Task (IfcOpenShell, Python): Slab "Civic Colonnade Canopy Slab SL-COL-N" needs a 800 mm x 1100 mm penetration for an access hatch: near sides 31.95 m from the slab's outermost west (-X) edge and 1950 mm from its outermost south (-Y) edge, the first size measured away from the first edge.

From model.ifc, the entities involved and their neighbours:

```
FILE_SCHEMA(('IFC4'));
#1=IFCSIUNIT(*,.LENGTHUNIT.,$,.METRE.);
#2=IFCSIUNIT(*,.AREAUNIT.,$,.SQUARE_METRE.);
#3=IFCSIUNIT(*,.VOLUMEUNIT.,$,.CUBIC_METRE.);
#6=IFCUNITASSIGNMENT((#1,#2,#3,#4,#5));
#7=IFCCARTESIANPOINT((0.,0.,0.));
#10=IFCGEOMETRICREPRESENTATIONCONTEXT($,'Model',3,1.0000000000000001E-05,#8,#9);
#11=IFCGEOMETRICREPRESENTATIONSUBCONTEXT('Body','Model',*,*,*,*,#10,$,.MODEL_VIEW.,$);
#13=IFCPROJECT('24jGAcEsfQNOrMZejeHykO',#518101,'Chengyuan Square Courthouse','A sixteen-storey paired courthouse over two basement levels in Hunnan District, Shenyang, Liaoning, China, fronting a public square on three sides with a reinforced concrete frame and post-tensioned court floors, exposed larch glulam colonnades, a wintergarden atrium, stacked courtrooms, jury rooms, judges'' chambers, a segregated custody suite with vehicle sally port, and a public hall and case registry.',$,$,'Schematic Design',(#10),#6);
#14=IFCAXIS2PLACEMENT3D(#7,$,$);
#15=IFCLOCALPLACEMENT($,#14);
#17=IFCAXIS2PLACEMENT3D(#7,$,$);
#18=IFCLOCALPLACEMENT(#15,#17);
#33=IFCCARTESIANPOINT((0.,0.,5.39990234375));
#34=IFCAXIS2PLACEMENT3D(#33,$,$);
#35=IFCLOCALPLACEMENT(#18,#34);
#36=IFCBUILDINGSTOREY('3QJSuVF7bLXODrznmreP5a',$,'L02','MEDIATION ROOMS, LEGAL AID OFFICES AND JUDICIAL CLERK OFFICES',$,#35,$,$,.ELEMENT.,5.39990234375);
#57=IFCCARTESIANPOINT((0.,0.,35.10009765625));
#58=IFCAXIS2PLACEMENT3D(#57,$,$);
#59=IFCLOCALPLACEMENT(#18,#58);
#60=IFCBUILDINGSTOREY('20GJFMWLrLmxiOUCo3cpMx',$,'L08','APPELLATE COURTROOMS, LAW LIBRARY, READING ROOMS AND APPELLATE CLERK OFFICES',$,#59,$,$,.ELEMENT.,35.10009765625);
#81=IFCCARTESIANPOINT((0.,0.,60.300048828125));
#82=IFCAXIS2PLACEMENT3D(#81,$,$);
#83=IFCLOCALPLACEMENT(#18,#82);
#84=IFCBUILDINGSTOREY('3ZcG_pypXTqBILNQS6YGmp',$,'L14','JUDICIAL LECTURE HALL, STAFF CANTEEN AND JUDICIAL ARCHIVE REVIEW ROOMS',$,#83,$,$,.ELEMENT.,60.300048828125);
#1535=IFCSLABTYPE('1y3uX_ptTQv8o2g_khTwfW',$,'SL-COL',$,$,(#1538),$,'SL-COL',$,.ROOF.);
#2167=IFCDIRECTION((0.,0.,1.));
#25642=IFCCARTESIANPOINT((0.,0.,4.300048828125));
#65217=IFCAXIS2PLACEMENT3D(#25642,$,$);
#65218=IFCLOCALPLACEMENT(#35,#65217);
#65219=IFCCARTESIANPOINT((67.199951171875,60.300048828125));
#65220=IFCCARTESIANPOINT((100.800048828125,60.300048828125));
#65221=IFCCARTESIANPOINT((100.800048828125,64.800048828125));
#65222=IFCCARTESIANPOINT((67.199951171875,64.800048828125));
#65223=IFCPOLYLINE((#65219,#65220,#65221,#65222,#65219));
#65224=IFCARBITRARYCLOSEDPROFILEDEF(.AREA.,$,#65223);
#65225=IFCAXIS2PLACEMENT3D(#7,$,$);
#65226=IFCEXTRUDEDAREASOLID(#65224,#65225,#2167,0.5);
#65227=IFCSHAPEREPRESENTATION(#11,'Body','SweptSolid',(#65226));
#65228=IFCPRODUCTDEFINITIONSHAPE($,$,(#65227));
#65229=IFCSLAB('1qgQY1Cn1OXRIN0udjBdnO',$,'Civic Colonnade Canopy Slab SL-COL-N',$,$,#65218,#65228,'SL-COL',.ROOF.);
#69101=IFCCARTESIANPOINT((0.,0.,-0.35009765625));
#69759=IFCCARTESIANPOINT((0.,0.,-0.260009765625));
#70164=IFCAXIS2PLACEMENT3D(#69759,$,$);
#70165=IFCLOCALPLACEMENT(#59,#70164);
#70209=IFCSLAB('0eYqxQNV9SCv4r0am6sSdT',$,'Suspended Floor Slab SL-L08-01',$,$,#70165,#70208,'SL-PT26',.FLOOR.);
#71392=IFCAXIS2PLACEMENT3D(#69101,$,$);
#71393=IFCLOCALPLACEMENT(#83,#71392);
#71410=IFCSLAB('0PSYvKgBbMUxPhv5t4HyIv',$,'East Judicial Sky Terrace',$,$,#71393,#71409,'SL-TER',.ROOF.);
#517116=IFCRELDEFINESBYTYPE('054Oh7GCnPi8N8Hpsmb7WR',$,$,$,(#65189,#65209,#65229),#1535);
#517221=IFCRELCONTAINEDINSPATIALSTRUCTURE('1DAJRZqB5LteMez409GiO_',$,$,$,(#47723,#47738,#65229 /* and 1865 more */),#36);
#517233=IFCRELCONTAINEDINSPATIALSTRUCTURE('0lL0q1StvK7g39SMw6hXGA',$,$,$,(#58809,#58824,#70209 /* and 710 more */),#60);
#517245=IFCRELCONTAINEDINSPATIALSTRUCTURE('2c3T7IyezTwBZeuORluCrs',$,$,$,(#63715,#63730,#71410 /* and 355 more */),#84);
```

```python
import numpy as np
import ifcopenshell
import ifcopenshell.api.feature
import ifcopenshell.api.geometry
import ifcopenshell.api.root
import ifcopenshell.geom
import ifcopenshell.util.placement
import ifcopenshell.util.representation
import ifcopenshell.util.shape
import ifcopenshell.util.unit

model = ifcopenshell.open("model.ifc")
unit_scale = ifcopenshell.util.unit.calculate_unit_scale(model)
settings = ifcopenshell.geom.settings()


def volume(element):
    """Net volume in cubic metres, openings subtracted."""
    shape = ifcopenshell.geom.create_shape(settings, element)
    return ifcopenshell.util.shape.get_volume(shape.geometry)


slab = model.by_guid("1qgQY1Cn1OXRIN0udjBdnO")
before = volume(slab)

# Extent in the slab's own axes, in metres. The edges named are its -X and -Y sides.
slab_shape = ifcopenshell.geom.create_shape(settings, slab)
vertices = ifcopenshell.util.shape.get_vertices(slab_shape.geometry)
x_min, y_min, bottom = vertices.min(axis=0)
top = vertices[:, 2].max()

opening = ifcopenshell.api.root.create_entity(model, ifc_class="IfcOpeningElement", name="Access hatch opening", predefined_type="OPENING")
context = ifcopenshell.util.representation.get_context(model, "Model", "Body", "MODEL_VIEW")
width, depth = 0.8, 1.1
outline = [(0.0, 0.0), (width, 0.0), (width, depth), (0.0, depth), (0.0, 0.0)]
# Overshoot both faces by 50 mm so the cut is clean.
shape = ifcopenshell.api.geometry.add_slab_representation(
    model, context=context, depth=top - bottom + 0.1, polyline=outline
)
ifcopenshell.api.geometry.assign_representation(model, product=opening, representation=shape)

matrix = ifcopenshell.util.placement.get_local_placement(slab.ObjectPlacement)
matrix[:, 3] = matrix @ np.append(np.array([x_min + 31.95, y_min + 1.95, bottom - 0.05]) / unit_scale, 1.0)
ifcopenshell.api.geometry.edit_object_placement(model, product=opening, matrix=matrix, is_si=False)
ifcopenshell.api.feature.add_feature(model, feature=opening, element=slab)

after = volume(slab)

print(f"slab volume {before:.3f} -> {after:.3f} m3")

model.write("model_edited.ifc")
```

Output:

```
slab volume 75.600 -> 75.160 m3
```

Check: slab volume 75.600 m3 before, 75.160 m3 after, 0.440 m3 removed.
